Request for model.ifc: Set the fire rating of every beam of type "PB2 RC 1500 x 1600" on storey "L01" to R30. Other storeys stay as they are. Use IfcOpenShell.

First a look at what the model holds.

```python
import ifcopenshell
import ifcopenshell.util.element

model = ifcopenshell.open("model.ifc")
print(model.schema)
storey = next(s for s in model.by_type("IfcBuildingStorey") if s.Name == "L01")
beams = [e for e in ifcopenshell.util.element.get_decomposition(storey) if e.is_a("IfcBeam")]
seen = {}
for e in beams:
    element_type = ifcopenshell.util.element.get_type(e)
    key = (element_type.Name if element_type != e and element_type else None, ifcopenshell.util.element.get_pset(e, "Pset_BeamCommon", "FireRating"))
    seen[key] = seen.get(key, 0) + 1
for (name, value), count in sorted(seen.items(), key=str):
    print(count, "x", name, "|", value)
```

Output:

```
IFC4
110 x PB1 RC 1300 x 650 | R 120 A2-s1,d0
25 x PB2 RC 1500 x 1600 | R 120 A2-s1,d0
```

```python
import ifcopenshell
import ifcopenshell.api.pset
import ifcopenshell.util.element

model = ifcopenshell.open("model.ifc")

storey = next(s for s in model.by_type("IfcBuildingStorey") if s.Name == "L01")
beams = [e for e in ifcopenshell.util.element.get_decomposition(storey) if e.is_a("IfcBeam")]

count = 0
for e in beams:
    element_type = ifcopenshell.util.element.get_type(e)
    if element_type in (None, e) or element_type.Name != "PB2 RC 1500 x 1600":
        continue
    found = ifcopenshell.util.element.get_pset(e, "Pset_BeamCommon", should_inherit=False)
    if found:
        pset = model.by_id(found["id"])
        if len(ifcopenshell.util.element.get_elements_by_pset(pset)) > 1:
            pset = ifcopenshell.api.pset.unshare_pset(model, products=[e], pset=pset)[0]
    else:
        pset = ifcopenshell.api.pset.add_pset(model, product=e, name="Pset_BeamCommon")
    ifcopenshell.api.pset.edit_pset(model, pset=pset, properties={"FireRating": "R30"})
    count += 1

print(count, "beams updated")

model.write("model-out.ifc")
```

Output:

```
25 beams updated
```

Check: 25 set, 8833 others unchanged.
